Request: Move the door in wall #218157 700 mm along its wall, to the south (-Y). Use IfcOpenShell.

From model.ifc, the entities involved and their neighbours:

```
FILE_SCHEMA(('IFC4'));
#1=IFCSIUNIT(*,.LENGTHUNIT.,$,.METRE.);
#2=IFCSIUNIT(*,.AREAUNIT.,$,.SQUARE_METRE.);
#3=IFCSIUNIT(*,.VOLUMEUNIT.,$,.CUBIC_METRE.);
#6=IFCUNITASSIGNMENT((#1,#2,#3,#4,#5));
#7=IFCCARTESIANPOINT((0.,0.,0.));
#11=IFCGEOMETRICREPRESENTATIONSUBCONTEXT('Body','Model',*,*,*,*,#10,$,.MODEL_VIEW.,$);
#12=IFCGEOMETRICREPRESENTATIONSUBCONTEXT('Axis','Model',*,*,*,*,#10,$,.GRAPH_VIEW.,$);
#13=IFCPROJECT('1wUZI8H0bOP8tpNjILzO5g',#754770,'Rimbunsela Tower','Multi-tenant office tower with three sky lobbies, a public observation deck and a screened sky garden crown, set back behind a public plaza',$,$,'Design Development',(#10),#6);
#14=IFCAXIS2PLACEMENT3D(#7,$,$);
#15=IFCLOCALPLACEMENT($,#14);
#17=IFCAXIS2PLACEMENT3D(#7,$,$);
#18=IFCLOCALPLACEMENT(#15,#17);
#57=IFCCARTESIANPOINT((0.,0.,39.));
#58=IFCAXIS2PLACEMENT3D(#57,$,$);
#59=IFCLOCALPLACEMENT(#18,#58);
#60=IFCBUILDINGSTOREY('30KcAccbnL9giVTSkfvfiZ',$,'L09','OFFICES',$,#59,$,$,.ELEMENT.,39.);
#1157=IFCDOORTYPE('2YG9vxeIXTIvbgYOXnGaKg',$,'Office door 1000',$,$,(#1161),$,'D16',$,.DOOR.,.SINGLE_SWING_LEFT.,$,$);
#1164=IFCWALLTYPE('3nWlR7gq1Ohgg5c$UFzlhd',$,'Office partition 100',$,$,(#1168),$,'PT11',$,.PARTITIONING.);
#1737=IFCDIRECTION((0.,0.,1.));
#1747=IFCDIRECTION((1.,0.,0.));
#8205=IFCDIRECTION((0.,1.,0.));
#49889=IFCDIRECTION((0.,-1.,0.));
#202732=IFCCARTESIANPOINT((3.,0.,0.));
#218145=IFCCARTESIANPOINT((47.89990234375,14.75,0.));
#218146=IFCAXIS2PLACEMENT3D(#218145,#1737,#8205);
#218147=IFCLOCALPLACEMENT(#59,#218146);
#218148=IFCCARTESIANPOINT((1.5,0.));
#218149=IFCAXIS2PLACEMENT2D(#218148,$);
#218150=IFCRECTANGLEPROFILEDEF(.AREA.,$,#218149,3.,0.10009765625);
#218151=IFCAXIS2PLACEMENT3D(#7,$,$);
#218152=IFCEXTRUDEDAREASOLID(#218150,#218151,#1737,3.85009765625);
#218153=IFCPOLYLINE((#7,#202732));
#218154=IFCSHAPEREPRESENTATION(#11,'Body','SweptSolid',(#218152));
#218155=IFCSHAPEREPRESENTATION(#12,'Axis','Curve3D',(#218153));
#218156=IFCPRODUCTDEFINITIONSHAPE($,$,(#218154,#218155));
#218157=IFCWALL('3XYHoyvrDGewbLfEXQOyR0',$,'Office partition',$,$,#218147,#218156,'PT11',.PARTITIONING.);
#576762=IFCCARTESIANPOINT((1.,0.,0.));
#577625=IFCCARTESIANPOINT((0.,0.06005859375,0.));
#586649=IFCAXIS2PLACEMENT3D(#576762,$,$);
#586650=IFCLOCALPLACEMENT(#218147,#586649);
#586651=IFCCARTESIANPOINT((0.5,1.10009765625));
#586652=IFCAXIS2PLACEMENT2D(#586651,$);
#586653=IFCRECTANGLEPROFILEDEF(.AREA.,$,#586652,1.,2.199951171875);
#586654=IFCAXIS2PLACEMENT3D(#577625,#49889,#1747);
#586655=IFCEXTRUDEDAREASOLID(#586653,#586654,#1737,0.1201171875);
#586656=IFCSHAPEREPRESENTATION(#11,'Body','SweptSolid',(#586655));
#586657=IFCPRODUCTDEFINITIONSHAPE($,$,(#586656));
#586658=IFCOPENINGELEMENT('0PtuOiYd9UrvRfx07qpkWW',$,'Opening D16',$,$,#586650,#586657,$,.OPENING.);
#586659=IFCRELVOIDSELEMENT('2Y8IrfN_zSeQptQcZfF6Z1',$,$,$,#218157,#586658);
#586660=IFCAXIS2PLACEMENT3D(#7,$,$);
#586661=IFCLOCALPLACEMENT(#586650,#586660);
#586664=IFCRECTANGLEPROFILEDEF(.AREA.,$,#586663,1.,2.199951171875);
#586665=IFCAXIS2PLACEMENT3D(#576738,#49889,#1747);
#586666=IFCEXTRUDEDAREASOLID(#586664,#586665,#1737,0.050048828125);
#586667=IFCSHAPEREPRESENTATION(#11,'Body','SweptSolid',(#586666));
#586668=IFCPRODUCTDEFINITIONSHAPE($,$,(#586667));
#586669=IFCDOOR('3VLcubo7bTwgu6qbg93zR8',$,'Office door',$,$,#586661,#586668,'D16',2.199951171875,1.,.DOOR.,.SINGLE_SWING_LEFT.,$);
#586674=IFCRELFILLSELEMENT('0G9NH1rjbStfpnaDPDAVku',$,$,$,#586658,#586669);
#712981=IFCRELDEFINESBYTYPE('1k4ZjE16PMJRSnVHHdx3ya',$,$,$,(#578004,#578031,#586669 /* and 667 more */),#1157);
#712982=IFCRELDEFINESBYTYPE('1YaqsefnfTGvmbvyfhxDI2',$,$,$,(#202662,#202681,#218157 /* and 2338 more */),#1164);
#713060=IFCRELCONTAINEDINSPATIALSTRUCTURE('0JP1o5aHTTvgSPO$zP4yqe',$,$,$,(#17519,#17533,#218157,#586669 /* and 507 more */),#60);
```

```python
import ifcopenshell
import ifcopenshell.api.geometry
import ifcopenshell.util.placement
import ifcopenshell.util.unit

model = ifcopenshell.open("model.ifc")
unit_scale = ifcopenshell.util.unit.calculate_unit_scale(model)

door = model.by_guid("3VLcubo7bTwgu6qbg93zR8")
opening = door.FillsVoids[0].RelatingOpeningElement
wall = opening.VoidsElements[0].RelatingBuildingElement

wall_matrix = ifcopenshell.util.placement.get_local_placement(wall.ObjectPlacement)
shift = wall_matrix[:3, 0] * -0.7 / unit_scale
before = ifcopenshell.util.placement.get_local_placement(door.ObjectPlacement)[:3, 3].copy()

# The door is placed relative to its opening, so it follows when the opening moves.
matrix = ifcopenshell.util.placement.get_local_placement(opening.ObjectPlacement)
matrix[:3, 3] += shift
ifcopenshell.api.geometry.edit_object_placement(
    model, product=opening, matrix=matrix, is_si=False, should_transform_children=True
)

after = ifcopenshell.util.placement.get_local_placement(door.ObjectPlacement)[:3, 3]
print("door moved by", (after - before).round(3) + 0.0)

model.write("model_rev.ifc")
```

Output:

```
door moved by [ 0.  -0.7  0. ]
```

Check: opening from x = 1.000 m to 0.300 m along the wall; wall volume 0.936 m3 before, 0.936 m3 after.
